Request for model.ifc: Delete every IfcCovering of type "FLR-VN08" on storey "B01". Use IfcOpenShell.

First a look at what the model holds.

```python
import ifcopenshell
import ifcopenshell.util.element

model = ifcopenshell.open("model.ifc")
print(model.schema)
storey = next(s for s in model.by_type("IfcBuildingStorey") if s.Name == "B01")
coverings = [e for e in ifcopenshell.util.element.get_decomposition(storey) if e.is_a("IfcCovering")]
seen = {}
for e in coverings:
    element_type = ifcopenshell.util.element.get_type(e)
    name = element_type.Name if element_type not in (None, e) else None
    seen[name] = seen.get(name, 0) + 1
for name, count in sorted(seen.items(), key=str):
    print(count, "x", name)
```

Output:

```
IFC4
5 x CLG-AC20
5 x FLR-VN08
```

```python
import ifcopenshell
import ifcopenshell.api.root
import ifcopenshell.util.element

model = ifcopenshell.open("model.ifc")

storey = next(s for s in model.by_type("IfcBuildingStorey") if s.Name == "B01")
coverings = [e for e in ifcopenshell.util.element.get_decomposition(storey) if e.is_a("IfcCovering")]
targets = [e for e in coverings if (t := ifcopenshell.util.element.get_type(e)) not in (None, e) and t.Name == "FLR-VN08"]

for e in targets:
    ifcopenshell.api.root.remove_product(model, product=e)
print(len(targets), "removed")

model.write("model_edited.ifc")
```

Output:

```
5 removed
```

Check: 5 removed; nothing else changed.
